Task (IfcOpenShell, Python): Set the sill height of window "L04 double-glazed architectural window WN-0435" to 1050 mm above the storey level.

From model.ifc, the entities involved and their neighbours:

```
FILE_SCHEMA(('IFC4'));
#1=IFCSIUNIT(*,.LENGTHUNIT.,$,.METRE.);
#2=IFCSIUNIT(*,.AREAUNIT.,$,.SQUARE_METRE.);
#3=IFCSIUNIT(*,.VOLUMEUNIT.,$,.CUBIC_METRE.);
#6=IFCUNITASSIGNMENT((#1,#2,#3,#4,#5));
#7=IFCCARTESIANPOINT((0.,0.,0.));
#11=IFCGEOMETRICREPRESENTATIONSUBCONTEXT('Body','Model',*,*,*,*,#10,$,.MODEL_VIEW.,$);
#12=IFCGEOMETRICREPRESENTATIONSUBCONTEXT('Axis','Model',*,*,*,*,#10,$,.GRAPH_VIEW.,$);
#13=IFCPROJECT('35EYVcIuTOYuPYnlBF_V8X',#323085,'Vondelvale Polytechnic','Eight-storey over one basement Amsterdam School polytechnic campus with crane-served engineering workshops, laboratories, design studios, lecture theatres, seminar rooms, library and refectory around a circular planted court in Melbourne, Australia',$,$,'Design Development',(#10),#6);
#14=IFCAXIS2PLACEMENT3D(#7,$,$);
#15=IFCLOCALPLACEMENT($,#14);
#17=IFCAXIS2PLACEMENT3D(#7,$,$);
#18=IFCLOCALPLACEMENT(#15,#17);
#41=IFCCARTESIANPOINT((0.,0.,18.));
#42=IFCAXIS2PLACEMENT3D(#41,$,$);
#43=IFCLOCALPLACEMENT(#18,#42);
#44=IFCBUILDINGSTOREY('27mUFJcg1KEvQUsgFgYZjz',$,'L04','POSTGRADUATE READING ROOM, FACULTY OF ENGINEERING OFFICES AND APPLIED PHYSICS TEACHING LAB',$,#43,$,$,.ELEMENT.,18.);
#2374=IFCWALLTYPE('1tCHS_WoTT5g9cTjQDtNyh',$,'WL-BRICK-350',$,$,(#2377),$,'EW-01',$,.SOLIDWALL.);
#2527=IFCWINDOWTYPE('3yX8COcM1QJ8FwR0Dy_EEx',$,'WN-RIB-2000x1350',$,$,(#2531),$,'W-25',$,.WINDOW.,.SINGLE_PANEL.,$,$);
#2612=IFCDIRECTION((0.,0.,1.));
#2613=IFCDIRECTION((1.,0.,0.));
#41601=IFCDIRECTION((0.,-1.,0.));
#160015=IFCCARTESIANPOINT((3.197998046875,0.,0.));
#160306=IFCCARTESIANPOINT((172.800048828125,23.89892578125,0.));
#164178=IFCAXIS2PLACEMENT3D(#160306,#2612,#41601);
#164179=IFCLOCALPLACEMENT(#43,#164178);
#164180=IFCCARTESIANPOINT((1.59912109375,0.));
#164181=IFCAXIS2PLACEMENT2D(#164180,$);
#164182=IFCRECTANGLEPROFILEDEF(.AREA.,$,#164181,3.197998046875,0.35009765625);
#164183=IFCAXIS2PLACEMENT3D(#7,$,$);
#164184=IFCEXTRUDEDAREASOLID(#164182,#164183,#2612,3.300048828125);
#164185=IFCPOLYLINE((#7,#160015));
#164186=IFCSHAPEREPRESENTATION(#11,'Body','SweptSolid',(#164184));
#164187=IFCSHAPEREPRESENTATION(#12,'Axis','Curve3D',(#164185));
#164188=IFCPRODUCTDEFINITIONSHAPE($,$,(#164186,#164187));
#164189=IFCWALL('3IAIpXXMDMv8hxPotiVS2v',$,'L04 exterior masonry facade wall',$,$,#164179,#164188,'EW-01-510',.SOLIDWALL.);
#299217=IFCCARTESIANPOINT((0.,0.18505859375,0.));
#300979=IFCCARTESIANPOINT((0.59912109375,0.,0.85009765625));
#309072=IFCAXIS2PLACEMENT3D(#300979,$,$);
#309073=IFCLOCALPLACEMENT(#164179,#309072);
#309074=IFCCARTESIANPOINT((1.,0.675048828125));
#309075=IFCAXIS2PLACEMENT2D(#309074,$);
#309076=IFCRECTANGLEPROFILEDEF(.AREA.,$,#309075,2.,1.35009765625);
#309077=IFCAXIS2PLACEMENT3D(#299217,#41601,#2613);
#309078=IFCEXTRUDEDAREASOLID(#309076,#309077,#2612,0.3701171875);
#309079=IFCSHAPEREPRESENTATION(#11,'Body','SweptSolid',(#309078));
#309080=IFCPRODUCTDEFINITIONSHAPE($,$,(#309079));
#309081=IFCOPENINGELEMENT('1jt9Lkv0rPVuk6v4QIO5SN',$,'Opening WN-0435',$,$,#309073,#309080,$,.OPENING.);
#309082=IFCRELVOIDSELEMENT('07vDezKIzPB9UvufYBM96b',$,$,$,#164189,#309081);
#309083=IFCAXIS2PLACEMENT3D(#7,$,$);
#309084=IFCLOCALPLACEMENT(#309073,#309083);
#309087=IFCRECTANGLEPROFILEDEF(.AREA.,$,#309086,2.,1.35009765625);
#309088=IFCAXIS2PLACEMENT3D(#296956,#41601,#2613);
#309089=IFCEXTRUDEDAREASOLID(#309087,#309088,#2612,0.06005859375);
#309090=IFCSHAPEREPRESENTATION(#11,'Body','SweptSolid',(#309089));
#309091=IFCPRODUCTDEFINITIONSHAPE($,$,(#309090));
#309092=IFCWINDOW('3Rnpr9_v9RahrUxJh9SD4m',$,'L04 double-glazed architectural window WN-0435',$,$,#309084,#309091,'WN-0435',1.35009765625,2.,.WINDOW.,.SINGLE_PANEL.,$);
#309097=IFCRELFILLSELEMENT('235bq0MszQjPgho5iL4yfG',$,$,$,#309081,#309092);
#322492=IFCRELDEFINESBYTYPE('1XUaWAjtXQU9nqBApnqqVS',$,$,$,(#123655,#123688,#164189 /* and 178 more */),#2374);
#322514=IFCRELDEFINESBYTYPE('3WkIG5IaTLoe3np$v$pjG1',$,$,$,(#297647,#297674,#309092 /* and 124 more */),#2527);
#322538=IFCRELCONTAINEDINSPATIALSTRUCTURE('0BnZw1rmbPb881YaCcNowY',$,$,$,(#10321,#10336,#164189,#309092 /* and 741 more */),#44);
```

```python
import numpy as np
import ifcopenshell
import ifcopenshell.api.geometry
import ifcopenshell.geom
import ifcopenshell.util.element
import ifcopenshell.util.placement
import ifcopenshell.util.shape
import ifcopenshell.util.unit

model = ifcopenshell.open("model.ifc")
unit_scale = ifcopenshell.util.unit.calculate_unit_scale(model)

window = model.by_guid("3Rnpr9_v9RahrUxJh9SD4m")
opening = window.FillsVoids[0].RelatingOpeningElement
storey = ifcopenshell.util.element.get_container(window, ifc_class="IfcBuildingStorey")
level = ifcopenshell.util.placement.get_local_placement(storey.ObjectPlacement)[2, 3]

# The opening's origin need not be at the sill, so measure its lowest point.
shape = ifcopenshell.geom.create_shape(ifcopenshell.geom.settings(), opening)
bottom = ifcopenshell.util.shape.get_shape_bottom_elevation(shape, shape.geometry) / unit_scale
dz = level + 1.05 / unit_scale - bottom

shift = np.array([0.0, 0.0, dz])
# The window is placed relative to its opening, so it follows when the opening moves.
matrix = ifcopenshell.util.placement.get_local_placement(opening.ObjectPlacement)
matrix[:3, 3] += shift
ifcopenshell.api.geometry.edit_object_placement(
    model, product=opening, matrix=matrix, is_si=False, should_transform_children=True
)

print(f"moved by {dz * unit_scale:+.3f} m")

model.write("model_edited.ifc")
```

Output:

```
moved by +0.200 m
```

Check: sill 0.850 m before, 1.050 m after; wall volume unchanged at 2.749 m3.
